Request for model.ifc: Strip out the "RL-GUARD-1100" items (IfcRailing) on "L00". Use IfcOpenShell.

First a look at what the model holds.

```python
import ifcopenshell
import ifcopenshell.util.element

model = ifcopenshell.open("model.ifc")
print(model.schema)
storey = next(s for s in model.by_type("IfcBuildingStorey") if s.Name == "L00")
railings = [e for e in ifcopenshell.util.element.get_decomposition(storey) if e.is_a("IfcRailing")]
seen = {}
for e in railings:
    element_type = ifcopenshell.util.element.get_type(e)
    name = element_type.Name if element_type not in (None, e) else None
    seen[name] = seen.get(name, 0) + 1
for name, count in sorted(seen.items(), key=str):
    print(count, "x", name)
```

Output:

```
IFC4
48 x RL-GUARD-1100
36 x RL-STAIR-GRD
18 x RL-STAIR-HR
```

```python
import ifcopenshell
import ifcopenshell.api.root
import ifcopenshell.util.element

model = ifcopenshell.open("model.ifc")

storey = next(s for s in model.by_type("IfcBuildingStorey") if s.Name == "L00")
railings = [e for e in ifcopenshell.util.element.get_decomposition(storey) if e.is_a("IfcRailing")]
targets = [e for e in railings if (t := ifcopenshell.util.element.get_type(e)) not in (None, e) and t.Name == "RL-GUARD-1100"]

for e in targets:
    ifcopenshell.api.root.remove_product(model, product=e)
print(len(targets), "removed")

model.write("model-out.ifc")
```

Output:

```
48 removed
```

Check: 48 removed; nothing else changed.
